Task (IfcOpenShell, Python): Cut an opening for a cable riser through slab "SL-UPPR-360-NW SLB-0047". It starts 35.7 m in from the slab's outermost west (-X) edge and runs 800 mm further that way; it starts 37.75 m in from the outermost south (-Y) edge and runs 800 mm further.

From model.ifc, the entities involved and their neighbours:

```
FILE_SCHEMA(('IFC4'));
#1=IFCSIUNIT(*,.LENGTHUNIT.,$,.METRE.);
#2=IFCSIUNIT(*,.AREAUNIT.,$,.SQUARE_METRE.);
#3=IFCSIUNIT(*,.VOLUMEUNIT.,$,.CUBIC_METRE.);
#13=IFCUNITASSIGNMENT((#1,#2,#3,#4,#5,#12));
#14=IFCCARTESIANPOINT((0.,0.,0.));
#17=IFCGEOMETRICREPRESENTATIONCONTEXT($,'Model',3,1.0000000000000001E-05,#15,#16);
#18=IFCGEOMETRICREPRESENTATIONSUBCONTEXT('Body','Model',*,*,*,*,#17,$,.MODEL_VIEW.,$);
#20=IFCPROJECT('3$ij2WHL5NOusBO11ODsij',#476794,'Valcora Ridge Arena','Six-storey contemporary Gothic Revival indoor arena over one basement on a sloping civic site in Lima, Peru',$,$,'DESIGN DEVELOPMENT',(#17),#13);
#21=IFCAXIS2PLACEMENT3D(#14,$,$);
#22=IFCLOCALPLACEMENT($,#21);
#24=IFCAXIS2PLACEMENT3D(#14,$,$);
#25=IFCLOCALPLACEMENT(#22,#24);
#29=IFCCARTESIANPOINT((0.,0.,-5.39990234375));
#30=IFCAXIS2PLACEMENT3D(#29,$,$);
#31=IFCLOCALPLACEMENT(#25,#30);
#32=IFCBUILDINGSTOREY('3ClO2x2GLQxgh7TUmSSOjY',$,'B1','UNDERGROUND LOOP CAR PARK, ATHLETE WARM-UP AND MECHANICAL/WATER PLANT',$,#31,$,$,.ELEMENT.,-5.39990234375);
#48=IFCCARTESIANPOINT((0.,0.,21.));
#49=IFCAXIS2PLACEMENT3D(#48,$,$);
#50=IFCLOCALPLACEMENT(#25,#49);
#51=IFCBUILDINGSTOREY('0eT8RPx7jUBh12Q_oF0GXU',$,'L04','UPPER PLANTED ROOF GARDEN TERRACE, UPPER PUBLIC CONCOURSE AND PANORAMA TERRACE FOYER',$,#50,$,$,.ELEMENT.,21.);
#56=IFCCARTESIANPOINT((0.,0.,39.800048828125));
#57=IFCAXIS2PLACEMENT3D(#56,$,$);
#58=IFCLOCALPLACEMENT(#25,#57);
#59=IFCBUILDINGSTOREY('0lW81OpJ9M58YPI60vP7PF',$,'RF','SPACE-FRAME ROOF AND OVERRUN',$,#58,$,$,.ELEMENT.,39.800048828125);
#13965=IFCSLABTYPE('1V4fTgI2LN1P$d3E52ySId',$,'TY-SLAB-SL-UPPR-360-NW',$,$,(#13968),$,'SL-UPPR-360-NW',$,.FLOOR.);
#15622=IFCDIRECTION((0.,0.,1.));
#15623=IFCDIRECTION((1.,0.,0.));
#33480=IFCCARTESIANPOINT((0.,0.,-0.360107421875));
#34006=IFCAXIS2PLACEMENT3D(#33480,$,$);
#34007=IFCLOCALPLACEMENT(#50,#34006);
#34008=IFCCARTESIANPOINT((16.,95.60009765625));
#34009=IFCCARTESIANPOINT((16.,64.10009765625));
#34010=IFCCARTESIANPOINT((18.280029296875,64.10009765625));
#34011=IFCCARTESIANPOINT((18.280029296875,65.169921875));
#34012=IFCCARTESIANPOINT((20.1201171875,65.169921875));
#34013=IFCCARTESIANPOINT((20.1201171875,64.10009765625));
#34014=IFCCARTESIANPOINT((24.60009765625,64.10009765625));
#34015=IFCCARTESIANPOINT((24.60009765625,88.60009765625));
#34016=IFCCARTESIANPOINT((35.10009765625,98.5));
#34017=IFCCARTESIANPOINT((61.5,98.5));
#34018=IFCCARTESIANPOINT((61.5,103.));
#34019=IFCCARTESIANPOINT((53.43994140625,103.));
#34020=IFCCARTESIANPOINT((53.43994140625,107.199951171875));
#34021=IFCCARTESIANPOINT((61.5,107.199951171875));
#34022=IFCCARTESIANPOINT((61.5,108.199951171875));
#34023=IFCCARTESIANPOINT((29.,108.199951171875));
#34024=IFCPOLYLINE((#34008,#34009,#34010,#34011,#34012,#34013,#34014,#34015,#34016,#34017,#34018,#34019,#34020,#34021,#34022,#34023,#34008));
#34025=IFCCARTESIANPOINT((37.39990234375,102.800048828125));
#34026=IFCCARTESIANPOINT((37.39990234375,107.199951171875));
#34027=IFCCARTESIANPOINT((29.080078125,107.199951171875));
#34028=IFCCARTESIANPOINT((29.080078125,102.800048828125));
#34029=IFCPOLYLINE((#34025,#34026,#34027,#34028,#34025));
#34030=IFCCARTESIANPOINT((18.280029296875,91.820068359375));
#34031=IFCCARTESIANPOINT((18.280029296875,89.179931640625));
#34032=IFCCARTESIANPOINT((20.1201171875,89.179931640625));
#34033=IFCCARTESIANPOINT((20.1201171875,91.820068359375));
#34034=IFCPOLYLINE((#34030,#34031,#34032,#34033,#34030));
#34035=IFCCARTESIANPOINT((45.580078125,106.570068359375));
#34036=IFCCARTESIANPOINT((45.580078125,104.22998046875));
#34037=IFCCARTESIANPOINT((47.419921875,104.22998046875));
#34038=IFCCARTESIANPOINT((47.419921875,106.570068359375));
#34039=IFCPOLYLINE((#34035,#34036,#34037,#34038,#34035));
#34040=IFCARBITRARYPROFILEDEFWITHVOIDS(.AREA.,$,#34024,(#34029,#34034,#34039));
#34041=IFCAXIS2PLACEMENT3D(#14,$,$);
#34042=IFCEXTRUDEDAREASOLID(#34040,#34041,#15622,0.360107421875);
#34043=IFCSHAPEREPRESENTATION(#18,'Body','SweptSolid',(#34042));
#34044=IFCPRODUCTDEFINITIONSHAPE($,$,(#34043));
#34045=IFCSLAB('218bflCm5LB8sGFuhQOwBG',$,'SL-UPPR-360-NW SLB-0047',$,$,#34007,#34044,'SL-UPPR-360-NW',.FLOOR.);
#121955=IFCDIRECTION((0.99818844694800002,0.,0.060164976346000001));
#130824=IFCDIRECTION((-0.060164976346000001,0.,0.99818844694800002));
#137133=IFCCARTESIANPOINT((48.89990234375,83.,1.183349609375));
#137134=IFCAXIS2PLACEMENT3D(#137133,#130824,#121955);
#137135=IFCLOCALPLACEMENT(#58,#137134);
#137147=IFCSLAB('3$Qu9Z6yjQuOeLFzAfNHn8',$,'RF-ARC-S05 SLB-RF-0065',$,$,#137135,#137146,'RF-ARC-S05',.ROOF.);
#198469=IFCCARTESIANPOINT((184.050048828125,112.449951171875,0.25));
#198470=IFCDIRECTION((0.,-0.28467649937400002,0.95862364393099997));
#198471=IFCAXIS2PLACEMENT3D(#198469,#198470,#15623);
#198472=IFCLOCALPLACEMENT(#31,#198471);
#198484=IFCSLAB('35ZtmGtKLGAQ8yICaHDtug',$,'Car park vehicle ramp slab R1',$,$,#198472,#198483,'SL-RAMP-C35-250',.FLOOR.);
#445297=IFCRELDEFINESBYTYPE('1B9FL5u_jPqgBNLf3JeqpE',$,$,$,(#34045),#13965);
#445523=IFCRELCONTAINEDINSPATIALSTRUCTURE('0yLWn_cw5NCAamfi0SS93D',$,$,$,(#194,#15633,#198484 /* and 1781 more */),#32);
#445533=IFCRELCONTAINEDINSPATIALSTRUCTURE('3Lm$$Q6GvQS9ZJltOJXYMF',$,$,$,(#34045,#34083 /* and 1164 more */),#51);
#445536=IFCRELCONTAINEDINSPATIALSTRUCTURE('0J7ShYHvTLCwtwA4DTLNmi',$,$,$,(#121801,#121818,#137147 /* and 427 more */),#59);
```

```python
import numpy as np
import ifcopenshell
import ifcopenshell.api.feature
import ifcopenshell.api.geometry
import ifcopenshell.api.root
import ifcopenshell.geom
import ifcopenshell.util.placement
import ifcopenshell.util.representation
import ifcopenshell.util.shape
import ifcopenshell.util.unit

model = ifcopenshell.open("model.ifc")
unit_scale = ifcopenshell.util.unit.calculate_unit_scale(model)
settings = ifcopenshell.geom.settings()


def volume(element):
    """Net volume in cubic metres, openings subtracted."""
    shape = ifcopenshell.geom.create_shape(settings, element)
    return ifcopenshell.util.shape.get_volume(shape.geometry)


slab = model.by_guid("218bflCm5LB8sGFuhQOwBG")
before = volume(slab)

# Extent in the slab's own axes, in metres. The edges named are its -X and -Y sides.
slab_shape = ifcopenshell.geom.create_shape(settings, slab)
vertices = ifcopenshell.util.shape.get_vertices(slab_shape.geometry)
x_min, y_min, bottom = vertices.min(axis=0)
top = vertices[:, 2].max()

opening = ifcopenshell.api.root.create_entity(model, ifc_class="IfcOpeningElement", name="Cable riser opening", predefined_type="OPENING")
context = ifcopenshell.util.representation.get_context(model, "Model", "Body", "MODEL_VIEW")
width, depth = 0.8, 0.8
outline = [(0.0, 0.0), (width, 0.0), (width, depth), (0.0, depth), (0.0, 0.0)]
# Overshoot both faces by 50 mm so the cut is clean.
shape = ifcopenshell.api.geometry.add_slab_representation(
    model, context=context, depth=top - bottom + 0.1, polyline=outline
)
ifcopenshell.api.geometry.assign_representation(model, product=opening, representation=shape)

matrix = ifcopenshell.util.placement.get_local_placement(slab.ObjectPlacement)
matrix[:, 3] = matrix @ np.append(np.array([x_min + 35.7, y_min + 37.75, bottom - 0.05]) / unit_scale, 1.0)
ifcopenshell.api.geometry.edit_object_placement(model, product=opening, matrix=matrix, is_si=False)
ifcopenshell.api.feature.add_feature(model, feature=opening, element=slab)

after = volume(slab)

print(f"slab volume {before:.3f} -> {after:.3f} m3")

model.write("model_v2.ifc")
```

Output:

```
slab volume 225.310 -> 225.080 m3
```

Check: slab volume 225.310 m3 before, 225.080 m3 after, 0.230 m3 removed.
